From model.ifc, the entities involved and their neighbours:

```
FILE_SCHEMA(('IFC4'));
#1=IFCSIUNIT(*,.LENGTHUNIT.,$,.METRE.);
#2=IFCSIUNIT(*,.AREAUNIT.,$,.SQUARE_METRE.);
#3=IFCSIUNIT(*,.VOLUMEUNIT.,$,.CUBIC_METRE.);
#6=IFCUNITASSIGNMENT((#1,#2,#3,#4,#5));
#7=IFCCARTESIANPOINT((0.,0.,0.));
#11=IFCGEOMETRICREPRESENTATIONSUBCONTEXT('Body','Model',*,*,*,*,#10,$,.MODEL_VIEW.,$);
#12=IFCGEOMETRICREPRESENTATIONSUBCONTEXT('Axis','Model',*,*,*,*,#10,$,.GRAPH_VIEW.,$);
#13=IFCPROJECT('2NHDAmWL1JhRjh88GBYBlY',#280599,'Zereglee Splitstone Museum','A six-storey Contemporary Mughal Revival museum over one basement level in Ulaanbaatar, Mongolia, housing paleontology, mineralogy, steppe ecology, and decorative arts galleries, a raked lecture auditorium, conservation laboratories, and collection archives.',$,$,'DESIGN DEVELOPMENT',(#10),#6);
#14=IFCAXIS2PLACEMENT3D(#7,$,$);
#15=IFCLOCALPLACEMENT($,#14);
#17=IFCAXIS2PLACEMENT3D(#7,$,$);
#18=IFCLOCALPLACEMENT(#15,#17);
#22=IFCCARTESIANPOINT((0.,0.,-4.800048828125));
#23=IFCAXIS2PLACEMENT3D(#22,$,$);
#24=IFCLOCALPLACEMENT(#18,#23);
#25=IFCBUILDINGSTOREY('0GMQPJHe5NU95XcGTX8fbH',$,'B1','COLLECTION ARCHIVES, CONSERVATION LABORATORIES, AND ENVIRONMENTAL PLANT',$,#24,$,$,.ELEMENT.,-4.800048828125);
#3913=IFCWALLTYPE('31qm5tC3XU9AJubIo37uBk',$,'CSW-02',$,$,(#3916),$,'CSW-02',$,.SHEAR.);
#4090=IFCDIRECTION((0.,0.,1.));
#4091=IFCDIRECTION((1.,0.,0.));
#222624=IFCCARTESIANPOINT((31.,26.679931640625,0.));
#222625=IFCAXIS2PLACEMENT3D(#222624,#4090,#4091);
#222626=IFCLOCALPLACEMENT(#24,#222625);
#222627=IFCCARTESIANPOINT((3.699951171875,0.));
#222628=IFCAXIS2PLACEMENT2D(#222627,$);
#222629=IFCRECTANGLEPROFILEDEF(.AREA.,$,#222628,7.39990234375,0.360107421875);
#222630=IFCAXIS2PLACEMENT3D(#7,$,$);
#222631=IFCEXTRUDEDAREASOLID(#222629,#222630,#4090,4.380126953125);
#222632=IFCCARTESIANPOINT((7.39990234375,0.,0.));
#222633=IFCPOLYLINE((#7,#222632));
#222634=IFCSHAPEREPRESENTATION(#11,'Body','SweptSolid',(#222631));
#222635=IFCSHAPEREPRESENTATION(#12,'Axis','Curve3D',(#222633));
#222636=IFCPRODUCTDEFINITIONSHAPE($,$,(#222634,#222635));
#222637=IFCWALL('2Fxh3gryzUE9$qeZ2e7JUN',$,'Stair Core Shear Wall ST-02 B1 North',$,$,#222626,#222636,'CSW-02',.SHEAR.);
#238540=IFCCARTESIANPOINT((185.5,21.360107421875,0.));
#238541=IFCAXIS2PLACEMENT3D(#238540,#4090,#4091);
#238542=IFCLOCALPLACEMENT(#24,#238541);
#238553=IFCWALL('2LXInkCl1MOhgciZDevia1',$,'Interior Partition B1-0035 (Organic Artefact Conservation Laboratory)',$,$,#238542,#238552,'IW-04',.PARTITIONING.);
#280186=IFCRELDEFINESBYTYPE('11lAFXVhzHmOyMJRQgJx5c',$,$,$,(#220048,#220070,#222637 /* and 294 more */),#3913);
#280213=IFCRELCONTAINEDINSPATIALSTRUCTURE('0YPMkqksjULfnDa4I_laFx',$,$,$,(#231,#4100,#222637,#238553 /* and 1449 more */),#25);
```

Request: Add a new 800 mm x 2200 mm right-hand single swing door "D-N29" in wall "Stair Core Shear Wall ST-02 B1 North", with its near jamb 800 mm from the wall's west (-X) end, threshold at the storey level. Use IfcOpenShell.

```python
import numpy as np
import ifcopenshell
import ifcopenshell.api.feature
import ifcopenshell.api.geometry
import ifcopenshell.api.root
import ifcopenshell.api.spatial
import ifcopenshell.geom
import ifcopenshell.util.element
import ifcopenshell.util.placement
import ifcopenshell.util.representation
import ifcopenshell.util.shape
import ifcopenshell.util.unit

model = ifcopenshell.open("model.ifc")
unit_scale = ifcopenshell.util.unit.calculate_unit_scale(model)
settings = ifcopenshell.geom.settings()


def volume(element):
    """Net volume in cubic metres, openings subtracted."""
    shape = ifcopenshell.geom.create_shape(settings, element)
    return ifcopenshell.util.shape.get_volume(shape.geometry)


wall = model.by_id(222637)
storey = ifcopenshell.util.element.get_container(wall, ifc_class="IfcBuildingStorey")
context = ifcopenshell.util.representation.get_context(model, "Model", "Body", "MODEL_VIEW")
before = volume(wall)

width, height, from_end, sill = 0.8, 2.2, 0.8, 0.0  # metres

# The wall runs along its own X axis, and the end named is its -X end.
wall_shape = ifcopenshell.geom.create_shape(settings, wall)
x, y, z = ifcopenshell.util.shape.get_vertices(wall_shape.geometry).T
start = x.min() + from_end
face, thickness = float(y.min()), float(y.max() - y.min())
wall_matrix = ifcopenshell.util.placement.get_local_placement(wall.ObjectPlacement)
level = ifcopenshell.util.placement.get_local_placement(storey.ObjectPlacement)[2, 3]


def in_wall(x, y):
    """Placement at x, y metres in the wall's axes, at sill height."""
    matrix = wall_matrix.copy()
    matrix[:, 3] = wall_matrix @ np.array([x / unit_scale, y / unit_scale, 0.0, 1.0])
    matrix[2, 3] = level + sill / unit_scale
    return matrix


# Opening: a box that overshoots both wall faces by 50 mm.
opening = ifcopenshell.api.root.create_entity(model, ifc_class="IfcOpeningElement", predefined_type="OPENING")
box = ifcopenshell.api.geometry.add_wall_representation(
    model, context=context, length=width, height=height, thickness=thickness + 0.1
)
ifcopenshell.api.geometry.assign_representation(model, product=opening, representation=box)
ifcopenshell.api.geometry.edit_object_placement(model, product=opening, matrix=in_wall(start, face - 0.05), is_si=False)
ifcopenshell.api.feature.add_feature(model, feature=opening, element=wall)

door = ifcopenshell.api.root.create_entity(model, ifc_class="IfcDoor", name="D-N29", predefined_type="DOOR")
door.OverallWidth, door.OverallHeight = width / unit_scale, height / unit_scale
door.OperationType = "SINGLE_SWING_RIGHT"
body = ifcopenshell.api.geometry.add_door_representation(
    model,
    context=context,
    overall_width=door.OverallWidth,
    overall_height=door.OverallHeight,
    operation_type="SINGLE_SWING_RIGHT",
    lining_properties={"LiningDepth": thickness / unit_scale, "ThresholdDepth": thickness / unit_scale},
)
ifcopenshell.api.geometry.assign_representation(model, product=door, representation=body)
ifcopenshell.api.spatial.assign_container(model, products=[door], relating_structure=storey)
ifcopenshell.api.feature.add_filling(model, opening=opening, element=door)

# The lining spans the wall, so the door starts at the wall face.
ifcopenshell.api.geometry.edit_object_placement(model, product=door, matrix=in_wall(start, face), is_si=False)

after = volume(wall)

print(f"wall volume {before:.3f} -> {after:.3f} m3")

model.write("model_edited.ifc")
```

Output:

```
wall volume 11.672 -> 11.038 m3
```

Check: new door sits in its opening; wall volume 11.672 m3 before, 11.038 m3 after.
